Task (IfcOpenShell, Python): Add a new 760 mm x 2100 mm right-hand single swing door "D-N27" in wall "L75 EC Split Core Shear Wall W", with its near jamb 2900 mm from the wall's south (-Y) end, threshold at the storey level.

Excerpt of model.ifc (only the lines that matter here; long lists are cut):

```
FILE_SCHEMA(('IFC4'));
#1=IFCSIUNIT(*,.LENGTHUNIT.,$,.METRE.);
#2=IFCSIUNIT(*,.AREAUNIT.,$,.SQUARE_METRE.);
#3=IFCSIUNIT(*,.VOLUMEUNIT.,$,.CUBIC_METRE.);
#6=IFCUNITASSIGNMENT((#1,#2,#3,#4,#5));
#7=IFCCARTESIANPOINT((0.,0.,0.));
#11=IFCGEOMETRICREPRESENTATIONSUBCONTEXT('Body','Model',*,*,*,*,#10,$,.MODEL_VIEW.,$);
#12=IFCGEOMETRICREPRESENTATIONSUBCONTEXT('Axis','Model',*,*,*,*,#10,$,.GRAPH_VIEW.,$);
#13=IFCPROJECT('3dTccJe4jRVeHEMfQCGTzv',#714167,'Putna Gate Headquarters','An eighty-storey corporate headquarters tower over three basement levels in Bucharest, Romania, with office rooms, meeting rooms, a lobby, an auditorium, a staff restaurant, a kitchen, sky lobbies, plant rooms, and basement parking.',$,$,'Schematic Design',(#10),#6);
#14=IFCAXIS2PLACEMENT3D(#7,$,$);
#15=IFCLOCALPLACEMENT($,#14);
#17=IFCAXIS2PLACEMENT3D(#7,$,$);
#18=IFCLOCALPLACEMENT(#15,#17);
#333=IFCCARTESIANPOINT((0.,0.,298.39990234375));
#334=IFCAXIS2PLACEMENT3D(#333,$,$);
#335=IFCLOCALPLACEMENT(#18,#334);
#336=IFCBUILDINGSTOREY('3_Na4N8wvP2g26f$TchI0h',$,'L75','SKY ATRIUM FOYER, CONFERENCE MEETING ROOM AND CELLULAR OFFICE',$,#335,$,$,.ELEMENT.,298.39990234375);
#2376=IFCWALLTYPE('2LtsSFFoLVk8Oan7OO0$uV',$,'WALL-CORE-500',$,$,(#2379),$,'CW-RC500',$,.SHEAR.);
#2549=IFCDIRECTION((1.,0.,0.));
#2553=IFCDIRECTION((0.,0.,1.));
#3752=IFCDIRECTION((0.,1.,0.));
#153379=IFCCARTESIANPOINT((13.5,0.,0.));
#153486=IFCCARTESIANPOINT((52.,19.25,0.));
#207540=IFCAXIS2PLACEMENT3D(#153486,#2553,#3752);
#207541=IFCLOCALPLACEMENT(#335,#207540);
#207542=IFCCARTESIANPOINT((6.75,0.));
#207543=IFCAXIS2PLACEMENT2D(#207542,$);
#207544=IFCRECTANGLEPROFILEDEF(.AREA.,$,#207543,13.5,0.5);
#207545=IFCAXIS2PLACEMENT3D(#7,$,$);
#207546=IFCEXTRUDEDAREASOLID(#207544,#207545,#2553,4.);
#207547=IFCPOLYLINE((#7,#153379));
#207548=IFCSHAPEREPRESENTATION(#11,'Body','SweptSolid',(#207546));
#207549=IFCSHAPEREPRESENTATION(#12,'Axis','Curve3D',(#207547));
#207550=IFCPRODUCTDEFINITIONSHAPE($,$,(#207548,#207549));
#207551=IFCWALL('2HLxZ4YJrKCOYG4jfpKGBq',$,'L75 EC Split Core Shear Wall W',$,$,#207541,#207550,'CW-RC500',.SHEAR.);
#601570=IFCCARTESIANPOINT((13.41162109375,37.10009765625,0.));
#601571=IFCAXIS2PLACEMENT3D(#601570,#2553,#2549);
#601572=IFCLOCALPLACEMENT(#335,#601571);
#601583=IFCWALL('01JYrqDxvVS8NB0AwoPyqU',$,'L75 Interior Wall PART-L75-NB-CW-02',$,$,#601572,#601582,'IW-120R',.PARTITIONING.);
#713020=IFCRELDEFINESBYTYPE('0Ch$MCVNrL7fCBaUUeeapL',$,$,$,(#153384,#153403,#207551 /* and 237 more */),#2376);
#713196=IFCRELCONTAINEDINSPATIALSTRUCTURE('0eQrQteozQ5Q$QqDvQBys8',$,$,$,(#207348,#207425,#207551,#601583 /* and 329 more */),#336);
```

```python
import numpy as np
import ifcopenshell
import ifcopenshell.api.feature
import ifcopenshell.api.geometry
import ifcopenshell.api.root
import ifcopenshell.api.spatial
import ifcopenshell.geom
import ifcopenshell.util.element
import ifcopenshell.util.placement
import ifcopenshell.util.representation
import ifcopenshell.util.shape
import ifcopenshell.util.unit

model = ifcopenshell.open("model.ifc")
unit_scale = ifcopenshell.util.unit.calculate_unit_scale(model)
settings = ifcopenshell.geom.settings()


def volume(element):
    """Net volume in cubic metres, openings subtracted."""
    shape = ifcopenshell.geom.create_shape(settings, element)
    return ifcopenshell.util.shape.get_volume(shape.geometry)


wall = model.by_guid("2HLxZ4YJrKCOYG4jfpKGBq")
storey = ifcopenshell.util.element.get_container(wall, ifc_class="IfcBuildingStorey")
context = ifcopenshell.util.representation.get_context(model, "Model", "Body", "MODEL_VIEW")
before = volume(wall)

width, height, from_end, sill = 0.76, 2.1, 2.9, 0.0  # metres

# The wall runs along its own X axis, and the end named is its -X end.
wall_shape = ifcopenshell.geom.create_shape(settings, wall)
x, y, z = ifcopenshell.util.shape.get_vertices(wall_shape.geometry).T
start = x.min() + from_end
face, thickness = float(y.min()), float(y.max() - y.min())
wall_matrix = ifcopenshell.util.placement.get_local_placement(wall.ObjectPlacement)
level = ifcopenshell.util.placement.get_local_placement(storey.ObjectPlacement)[2, 3]


def in_wall(x, y):
    """Placement at x, y metres in the wall's axes, at sill height."""
    matrix = wall_matrix.copy()
    matrix[:, 3] = wall_matrix @ np.array([x / unit_scale, y / unit_scale, 0.0, 1.0])
    matrix[2, 3] = level + sill / unit_scale
    return matrix


# Opening: a box that overshoots both wall faces by 50 mm.
opening = ifcopenshell.api.root.create_entity(model, ifc_class="IfcOpeningElement", predefined_type="OPENING")
box = ifcopenshell.api.geometry.add_wall_representation(
    model, context=context, length=width, height=height, thickness=thickness + 0.1
)
ifcopenshell.api.geometry.assign_representation(model, product=opening, representation=box)
ifcopenshell.api.geometry.edit_object_placement(model, product=opening, matrix=in_wall(start, face - 0.05), is_si=False)
ifcopenshell.api.feature.add_feature(model, feature=opening, element=wall)

door = ifcopenshell.api.root.create_entity(model, ifc_class="IfcDoor", name="D-N27", predefined_type="DOOR")
door.OverallWidth, door.OverallHeight = width / unit_scale, height / unit_scale
door.OperationType = "SINGLE_SWING_RIGHT"
body = ifcopenshell.api.geometry.add_door_representation(
    model,
    context=context,
    overall_width=door.OverallWidth,
    overall_height=door.OverallHeight,
    operation_type="SINGLE_SWING_RIGHT",
    lining_properties={"LiningDepth": thickness / unit_scale, "ThresholdDepth": thickness / unit_scale},
)
ifcopenshell.api.geometry.assign_representation(model, product=door, representation=body)
ifcopenshell.api.spatial.assign_container(model, products=[door], relating_structure=storey)
ifcopenshell.api.feature.add_filling(model, opening=opening, element=door)

# The lining spans the wall, so the door starts at the wall face.
ifcopenshell.api.geometry.edit_object_placement(model, product=door, matrix=in_wall(start, face), is_si=False)

after = volume(wall)

print(f"wall volume {before:.3f} -> {after:.3f} m3")

model.write("model_rev.ifc")
```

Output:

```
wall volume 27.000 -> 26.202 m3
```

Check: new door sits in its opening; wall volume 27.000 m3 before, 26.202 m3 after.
